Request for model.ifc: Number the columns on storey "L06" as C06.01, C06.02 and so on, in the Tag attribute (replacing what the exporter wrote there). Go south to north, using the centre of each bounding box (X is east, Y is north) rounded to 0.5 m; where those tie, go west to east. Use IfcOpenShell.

First a look at what the model holds.

```python
import ifcopenshell
import ifcopenshell.util.element
import ifcopenshell.util.placement

model = ifcopenshell.open("model.ifc")
print(model.schema)
storey = next(s for s in model.by_type("IfcBuildingStorey") if s.Name == "L06")
columns = [e for e in ifcopenshell.util.element.get_decomposition(storey) if e.is_a("IfcColumn")]
for e in sorted(columns, key=lambda e: e.id()):
    origin = ifcopenshell.util.placement.get_local_placement(e.ObjectPlacement)[:3, 3]
    print(e.id(), e.Tag, e.Name, origin.round(2) + 0.0, sep=" | ")
```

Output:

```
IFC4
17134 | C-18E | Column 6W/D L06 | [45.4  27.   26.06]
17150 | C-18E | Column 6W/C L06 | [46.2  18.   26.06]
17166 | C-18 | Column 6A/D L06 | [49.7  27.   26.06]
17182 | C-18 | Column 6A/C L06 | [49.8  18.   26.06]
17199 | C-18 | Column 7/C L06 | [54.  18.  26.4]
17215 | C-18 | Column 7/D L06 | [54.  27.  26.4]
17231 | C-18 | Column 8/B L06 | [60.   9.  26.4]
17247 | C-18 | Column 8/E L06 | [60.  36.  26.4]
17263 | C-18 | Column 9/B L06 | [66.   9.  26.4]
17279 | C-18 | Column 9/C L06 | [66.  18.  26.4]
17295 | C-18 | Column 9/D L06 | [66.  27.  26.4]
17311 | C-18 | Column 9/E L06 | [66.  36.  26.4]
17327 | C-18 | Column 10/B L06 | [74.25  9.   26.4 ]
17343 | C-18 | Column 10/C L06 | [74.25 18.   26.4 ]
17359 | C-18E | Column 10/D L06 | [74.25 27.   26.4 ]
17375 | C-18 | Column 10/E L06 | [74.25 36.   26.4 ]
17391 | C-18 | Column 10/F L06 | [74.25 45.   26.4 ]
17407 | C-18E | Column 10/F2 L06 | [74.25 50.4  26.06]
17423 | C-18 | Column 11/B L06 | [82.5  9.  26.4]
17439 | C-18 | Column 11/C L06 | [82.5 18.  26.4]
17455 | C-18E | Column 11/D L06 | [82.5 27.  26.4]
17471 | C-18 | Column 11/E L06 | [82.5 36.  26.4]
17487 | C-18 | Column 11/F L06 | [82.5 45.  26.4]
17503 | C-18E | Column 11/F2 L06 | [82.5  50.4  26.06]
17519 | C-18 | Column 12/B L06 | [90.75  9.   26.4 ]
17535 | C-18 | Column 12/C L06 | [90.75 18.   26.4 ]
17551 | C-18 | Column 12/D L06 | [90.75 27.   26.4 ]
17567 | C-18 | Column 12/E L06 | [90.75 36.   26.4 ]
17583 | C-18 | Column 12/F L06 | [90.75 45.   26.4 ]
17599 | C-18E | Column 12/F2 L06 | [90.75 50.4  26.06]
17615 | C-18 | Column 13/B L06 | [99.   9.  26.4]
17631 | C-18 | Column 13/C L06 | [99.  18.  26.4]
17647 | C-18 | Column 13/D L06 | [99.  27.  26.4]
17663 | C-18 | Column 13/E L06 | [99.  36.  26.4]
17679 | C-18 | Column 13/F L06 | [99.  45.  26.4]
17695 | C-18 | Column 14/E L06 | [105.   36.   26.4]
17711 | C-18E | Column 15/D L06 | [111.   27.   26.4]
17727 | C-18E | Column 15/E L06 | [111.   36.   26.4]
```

```python
import ifcopenshell
import ifcopenshell.geom
import ifcopenshell.util.element
import ifcopenshell.util.shape

model = ifcopenshell.open("model.ifc")
settings = ifcopenshell.geom.settings()
settings.set("use-world-coords", True)


def centre(element):
    shape = ifcopenshell.geom.create_shape(settings, element)
    return ifcopenshell.util.shape.get_bbox_centroid(shape.geometry)


storey = next(s for s in model.by_type("IfcBuildingStorey") if s.Name == "L06")
columns = [e for e in ifcopenshell.util.element.get_decomposition(storey) if e.is_a("IfcColumn")]

# Insertion points can sit at a corner or the storey origin, so sort by the geometry (in metres).
centres = {e: centre(e) for e in columns}
columns.sort(key=lambda e: (round(centres[e][1] / 0.5), centres[e][0]))

for i, e in enumerate(columns, start=1):
    number = f"C06.{i:02d}"
    e.Tag = number
    print(e.id(), number)

model.write("model_v2.ifc")
```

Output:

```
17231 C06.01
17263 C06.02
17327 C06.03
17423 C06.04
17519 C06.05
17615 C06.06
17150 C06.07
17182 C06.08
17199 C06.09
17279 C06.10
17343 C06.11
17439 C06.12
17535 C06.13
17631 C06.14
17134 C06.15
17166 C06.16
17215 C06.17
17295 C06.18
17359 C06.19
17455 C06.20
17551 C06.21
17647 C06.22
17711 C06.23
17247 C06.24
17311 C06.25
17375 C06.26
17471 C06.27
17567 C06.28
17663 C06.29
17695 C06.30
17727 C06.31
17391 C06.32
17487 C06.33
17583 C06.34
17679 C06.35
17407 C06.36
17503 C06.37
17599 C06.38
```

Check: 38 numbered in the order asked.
